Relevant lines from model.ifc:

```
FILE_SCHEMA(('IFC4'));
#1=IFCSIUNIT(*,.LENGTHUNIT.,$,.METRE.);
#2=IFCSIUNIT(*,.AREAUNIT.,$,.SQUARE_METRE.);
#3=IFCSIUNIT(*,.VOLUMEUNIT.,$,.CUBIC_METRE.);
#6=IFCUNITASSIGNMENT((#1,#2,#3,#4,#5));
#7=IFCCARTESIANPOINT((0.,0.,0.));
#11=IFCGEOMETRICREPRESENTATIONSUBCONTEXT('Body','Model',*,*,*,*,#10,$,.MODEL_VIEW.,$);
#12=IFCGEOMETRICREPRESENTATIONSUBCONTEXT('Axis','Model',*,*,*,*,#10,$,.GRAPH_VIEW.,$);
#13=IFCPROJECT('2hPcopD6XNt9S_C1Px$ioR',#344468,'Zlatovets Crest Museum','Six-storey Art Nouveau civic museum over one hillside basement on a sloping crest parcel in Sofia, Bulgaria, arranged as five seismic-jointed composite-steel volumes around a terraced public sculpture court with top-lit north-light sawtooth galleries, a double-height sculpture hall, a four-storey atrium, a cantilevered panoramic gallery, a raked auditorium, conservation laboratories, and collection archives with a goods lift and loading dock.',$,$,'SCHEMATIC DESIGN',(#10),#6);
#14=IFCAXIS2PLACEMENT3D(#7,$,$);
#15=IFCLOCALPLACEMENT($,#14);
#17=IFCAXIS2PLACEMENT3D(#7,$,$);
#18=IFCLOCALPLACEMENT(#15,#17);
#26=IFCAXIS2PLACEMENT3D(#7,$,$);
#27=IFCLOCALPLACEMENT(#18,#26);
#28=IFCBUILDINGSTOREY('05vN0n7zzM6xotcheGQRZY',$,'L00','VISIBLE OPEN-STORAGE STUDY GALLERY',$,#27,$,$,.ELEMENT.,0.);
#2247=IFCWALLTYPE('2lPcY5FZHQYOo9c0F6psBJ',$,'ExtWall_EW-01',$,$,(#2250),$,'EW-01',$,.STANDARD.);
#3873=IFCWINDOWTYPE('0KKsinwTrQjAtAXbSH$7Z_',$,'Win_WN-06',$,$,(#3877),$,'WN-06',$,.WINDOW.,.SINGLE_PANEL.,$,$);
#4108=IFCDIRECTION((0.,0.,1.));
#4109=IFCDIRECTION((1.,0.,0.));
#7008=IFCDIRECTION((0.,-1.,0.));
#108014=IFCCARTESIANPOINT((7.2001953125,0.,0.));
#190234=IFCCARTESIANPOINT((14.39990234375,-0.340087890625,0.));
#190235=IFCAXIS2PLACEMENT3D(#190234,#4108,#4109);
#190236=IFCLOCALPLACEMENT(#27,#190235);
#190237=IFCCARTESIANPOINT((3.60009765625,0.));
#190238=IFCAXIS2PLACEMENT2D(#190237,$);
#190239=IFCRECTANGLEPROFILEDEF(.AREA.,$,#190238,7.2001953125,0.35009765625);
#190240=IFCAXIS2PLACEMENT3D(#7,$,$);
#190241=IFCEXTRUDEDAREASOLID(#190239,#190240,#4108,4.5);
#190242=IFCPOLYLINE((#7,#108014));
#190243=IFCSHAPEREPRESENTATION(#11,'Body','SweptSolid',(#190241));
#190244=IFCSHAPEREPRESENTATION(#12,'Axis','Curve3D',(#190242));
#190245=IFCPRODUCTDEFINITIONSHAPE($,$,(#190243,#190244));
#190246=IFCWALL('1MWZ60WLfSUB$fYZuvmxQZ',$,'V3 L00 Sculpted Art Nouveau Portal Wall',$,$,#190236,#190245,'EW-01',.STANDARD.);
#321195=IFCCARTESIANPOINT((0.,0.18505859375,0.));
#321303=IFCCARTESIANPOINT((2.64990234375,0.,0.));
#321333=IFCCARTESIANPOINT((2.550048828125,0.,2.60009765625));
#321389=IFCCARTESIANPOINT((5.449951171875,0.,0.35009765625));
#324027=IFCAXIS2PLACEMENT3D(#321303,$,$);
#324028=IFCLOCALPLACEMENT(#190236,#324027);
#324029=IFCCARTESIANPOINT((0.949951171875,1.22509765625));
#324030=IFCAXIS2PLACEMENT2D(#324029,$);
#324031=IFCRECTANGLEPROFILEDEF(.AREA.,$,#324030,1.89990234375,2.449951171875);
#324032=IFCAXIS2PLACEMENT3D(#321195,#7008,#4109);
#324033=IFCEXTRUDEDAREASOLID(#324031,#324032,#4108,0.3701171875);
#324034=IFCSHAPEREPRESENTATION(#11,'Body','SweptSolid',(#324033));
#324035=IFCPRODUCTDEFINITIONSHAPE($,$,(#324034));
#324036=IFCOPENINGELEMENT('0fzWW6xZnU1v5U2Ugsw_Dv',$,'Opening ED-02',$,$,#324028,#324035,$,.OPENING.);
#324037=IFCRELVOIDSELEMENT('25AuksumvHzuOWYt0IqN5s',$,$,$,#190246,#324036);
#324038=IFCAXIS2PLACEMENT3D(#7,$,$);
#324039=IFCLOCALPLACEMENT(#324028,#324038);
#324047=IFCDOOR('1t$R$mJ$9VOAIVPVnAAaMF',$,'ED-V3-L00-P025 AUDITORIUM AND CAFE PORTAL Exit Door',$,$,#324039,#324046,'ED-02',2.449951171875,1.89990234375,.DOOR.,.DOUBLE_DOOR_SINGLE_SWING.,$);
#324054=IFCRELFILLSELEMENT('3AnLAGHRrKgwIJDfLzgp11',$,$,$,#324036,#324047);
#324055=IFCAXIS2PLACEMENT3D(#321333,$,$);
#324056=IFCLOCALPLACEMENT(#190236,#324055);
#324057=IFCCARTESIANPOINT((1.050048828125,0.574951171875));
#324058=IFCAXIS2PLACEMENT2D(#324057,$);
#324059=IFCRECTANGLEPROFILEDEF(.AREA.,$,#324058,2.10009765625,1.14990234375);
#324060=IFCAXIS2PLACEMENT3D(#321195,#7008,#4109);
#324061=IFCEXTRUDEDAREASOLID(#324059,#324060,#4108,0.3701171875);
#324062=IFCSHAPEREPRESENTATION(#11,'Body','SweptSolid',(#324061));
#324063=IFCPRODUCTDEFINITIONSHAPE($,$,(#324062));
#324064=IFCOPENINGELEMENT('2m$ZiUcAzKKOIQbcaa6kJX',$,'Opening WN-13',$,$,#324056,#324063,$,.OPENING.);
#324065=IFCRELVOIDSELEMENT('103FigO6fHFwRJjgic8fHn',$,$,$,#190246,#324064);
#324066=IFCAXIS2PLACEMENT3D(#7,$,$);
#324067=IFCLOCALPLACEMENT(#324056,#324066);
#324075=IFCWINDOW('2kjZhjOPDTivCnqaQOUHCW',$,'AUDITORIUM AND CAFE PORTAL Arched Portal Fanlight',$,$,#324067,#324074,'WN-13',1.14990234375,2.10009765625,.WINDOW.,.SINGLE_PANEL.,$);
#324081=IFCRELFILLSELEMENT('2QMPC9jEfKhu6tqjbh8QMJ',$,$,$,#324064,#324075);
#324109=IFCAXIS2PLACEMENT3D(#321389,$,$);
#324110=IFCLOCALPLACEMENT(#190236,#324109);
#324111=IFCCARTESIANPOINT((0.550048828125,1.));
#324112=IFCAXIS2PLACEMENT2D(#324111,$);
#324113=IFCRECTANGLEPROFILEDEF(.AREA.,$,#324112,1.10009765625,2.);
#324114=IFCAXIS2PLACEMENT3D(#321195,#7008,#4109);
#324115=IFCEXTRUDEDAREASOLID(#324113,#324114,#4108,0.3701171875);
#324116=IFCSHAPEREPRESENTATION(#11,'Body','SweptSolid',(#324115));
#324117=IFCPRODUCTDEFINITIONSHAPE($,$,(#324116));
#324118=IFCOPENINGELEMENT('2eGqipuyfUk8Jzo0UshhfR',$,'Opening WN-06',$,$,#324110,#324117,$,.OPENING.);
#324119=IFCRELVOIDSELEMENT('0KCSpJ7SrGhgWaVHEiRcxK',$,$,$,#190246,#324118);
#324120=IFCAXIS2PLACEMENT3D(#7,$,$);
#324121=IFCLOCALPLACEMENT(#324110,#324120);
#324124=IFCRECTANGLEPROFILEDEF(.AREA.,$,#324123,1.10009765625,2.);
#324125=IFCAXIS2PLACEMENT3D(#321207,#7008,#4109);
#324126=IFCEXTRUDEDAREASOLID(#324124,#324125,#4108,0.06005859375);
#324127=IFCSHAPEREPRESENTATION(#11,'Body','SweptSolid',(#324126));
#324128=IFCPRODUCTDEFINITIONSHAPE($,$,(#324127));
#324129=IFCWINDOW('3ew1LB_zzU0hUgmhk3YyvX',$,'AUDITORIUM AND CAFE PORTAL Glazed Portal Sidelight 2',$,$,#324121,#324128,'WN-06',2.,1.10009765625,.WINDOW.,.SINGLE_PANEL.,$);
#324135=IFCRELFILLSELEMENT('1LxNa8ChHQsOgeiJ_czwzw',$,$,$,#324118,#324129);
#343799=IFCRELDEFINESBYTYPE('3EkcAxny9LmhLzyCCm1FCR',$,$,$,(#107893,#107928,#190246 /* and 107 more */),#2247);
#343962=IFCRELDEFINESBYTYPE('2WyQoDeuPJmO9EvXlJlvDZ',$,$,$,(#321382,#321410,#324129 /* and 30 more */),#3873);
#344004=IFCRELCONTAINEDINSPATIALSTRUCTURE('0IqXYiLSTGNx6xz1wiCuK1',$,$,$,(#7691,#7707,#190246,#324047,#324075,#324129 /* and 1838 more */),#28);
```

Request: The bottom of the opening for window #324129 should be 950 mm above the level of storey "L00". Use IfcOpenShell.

```python
import numpy as np
import ifcopenshell
import ifcopenshell.api.geometry
import ifcopenshell.geom
import ifcopenshell.util.element
import ifcopenshell.util.placement
import ifcopenshell.util.shape
import ifcopenshell.util.unit

model = ifcopenshell.open("model.ifc")
unit_scale = ifcopenshell.util.unit.calculate_unit_scale(model)

window = model.by_guid("3ew1LB_zzU0hUgmhk3YyvX")
opening = window.FillsVoids[0].RelatingOpeningElement
storey = ifcopenshell.util.element.get_container(window, ifc_class="IfcBuildingStorey")
level = ifcopenshell.util.placement.get_local_placement(storey.ObjectPlacement)[2, 3]

# The opening's origin need not be at the sill, so measure its lowest point.
shape = ifcopenshell.geom.create_shape(ifcopenshell.geom.settings(), opening)
bottom = ifcopenshell.util.shape.get_shape_bottom_elevation(shape, shape.geometry) / unit_scale
dz = level + 0.95 / unit_scale - bottom

shift = np.array([0.0, 0.0, dz])
# The window is placed relative to its opening, so it follows when the opening moves.
matrix = ifcopenshell.util.placement.get_local_placement(opening.ObjectPlacement)
matrix[:3, 3] += shift
ifcopenshell.api.geometry.edit_object_placement(
    model, product=opening, matrix=matrix, is_si=False, should_transform_children=True
)

print(f"moved by {dz * unit_scale:+.3f} m")

model.write("model_rev.ifc")
```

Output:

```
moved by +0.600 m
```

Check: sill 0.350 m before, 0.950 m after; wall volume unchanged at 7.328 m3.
